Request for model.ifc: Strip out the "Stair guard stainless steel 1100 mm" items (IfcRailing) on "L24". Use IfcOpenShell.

First a look at what the model holds.

```python
import ifcopenshell
import ifcopenshell.util.element

model = ifcopenshell.open("model.ifc")
print(model.schema)
storey = next(s for s in model.by_type("IfcBuildingStorey") if s.Name == "L24")
railings = [e for e in ifcopenshell.util.element.get_decomposition(storey) if e.is_a("IfcRailing")]
seen = {}
for e in railings:
    element_type = ifcopenshell.util.element.get_type(e)
    name = element_type.Name if element_type not in (None, e) else None
    seen[name] = seen.get(name, 0) + 1
for name, count in sorted(seen.items(), key=str):
    print(count, "x", name)
```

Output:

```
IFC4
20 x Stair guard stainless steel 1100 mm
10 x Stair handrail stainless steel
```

```python
import ifcopenshell
import ifcopenshell.api.root
import ifcopenshell.util.element

model = ifcopenshell.open("model.ifc")

storey = next(s for s in model.by_type("IfcBuildingStorey") if s.Name == "L24")
railings = [e for e in ifcopenshell.util.element.get_decomposition(storey) if e.is_a("IfcRailing")]
targets = [e for e in railings if (t := ifcopenshell.util.element.get_type(e)) not in (None, e) and t.Name == "Stair guard stainless steel 1100 mm"]

for e in targets:
    ifcopenshell.api.root.remove_product(model, product=e)
print(len(targets), "removed")

model.write("model_rev.ifc")
```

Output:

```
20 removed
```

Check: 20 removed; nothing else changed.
